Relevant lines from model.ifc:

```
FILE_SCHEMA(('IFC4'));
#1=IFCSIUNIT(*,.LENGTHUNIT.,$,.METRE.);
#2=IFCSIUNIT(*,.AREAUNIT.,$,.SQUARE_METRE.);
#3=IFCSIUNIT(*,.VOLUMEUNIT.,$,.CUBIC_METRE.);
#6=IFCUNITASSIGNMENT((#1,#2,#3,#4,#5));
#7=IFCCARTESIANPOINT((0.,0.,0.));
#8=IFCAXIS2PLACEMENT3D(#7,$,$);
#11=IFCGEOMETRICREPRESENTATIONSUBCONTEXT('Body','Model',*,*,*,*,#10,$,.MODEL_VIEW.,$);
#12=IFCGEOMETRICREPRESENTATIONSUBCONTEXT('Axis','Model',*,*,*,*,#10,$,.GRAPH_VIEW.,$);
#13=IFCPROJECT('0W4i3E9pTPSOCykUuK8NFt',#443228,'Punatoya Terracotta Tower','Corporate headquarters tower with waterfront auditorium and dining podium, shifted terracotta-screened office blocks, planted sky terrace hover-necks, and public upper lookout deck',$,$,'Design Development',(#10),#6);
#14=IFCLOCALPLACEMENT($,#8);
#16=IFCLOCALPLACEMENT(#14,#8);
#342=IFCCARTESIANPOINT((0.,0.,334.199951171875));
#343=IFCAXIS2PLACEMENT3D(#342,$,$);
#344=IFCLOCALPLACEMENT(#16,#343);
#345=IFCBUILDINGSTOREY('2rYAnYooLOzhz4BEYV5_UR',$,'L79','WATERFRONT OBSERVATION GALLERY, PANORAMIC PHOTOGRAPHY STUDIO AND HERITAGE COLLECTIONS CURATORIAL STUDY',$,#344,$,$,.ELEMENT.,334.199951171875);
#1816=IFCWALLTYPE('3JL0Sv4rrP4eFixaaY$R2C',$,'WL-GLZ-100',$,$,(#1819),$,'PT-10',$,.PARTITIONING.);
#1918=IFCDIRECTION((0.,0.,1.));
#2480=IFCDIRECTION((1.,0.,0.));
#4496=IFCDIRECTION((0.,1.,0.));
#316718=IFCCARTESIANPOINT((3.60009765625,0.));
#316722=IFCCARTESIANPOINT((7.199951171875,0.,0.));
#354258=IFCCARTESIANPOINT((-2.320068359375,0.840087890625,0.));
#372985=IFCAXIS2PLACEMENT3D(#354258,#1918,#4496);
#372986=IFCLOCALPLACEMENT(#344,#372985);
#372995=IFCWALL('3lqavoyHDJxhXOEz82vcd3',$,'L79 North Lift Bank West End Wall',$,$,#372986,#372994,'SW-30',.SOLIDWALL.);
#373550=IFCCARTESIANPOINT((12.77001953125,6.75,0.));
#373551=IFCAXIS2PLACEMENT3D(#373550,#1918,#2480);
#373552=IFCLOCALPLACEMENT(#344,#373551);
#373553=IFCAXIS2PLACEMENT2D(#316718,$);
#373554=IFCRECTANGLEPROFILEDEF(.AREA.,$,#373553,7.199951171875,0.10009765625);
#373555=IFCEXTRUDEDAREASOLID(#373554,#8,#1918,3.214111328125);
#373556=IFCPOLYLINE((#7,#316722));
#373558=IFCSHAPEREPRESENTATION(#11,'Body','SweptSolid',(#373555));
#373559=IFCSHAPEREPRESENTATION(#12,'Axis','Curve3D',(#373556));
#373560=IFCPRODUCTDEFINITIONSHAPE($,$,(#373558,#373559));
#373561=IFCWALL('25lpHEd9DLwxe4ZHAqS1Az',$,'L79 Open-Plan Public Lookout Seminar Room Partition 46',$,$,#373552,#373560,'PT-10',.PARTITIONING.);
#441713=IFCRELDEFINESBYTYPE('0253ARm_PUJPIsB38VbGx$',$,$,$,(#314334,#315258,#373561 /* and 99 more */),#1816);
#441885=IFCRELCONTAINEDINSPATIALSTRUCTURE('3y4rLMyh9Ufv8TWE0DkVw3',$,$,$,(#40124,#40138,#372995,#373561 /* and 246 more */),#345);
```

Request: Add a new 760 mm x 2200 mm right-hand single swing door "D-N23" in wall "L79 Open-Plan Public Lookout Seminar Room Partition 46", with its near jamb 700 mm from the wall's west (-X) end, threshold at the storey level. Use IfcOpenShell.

```python
import numpy as np
import ifcopenshell
import ifcopenshell.api.feature
import ifcopenshell.api.geometry
import ifcopenshell.api.root
import ifcopenshell.api.spatial
import ifcopenshell.geom
import ifcopenshell.util.element
import ifcopenshell.util.placement
import ifcopenshell.util.representation
import ifcopenshell.util.shape
import ifcopenshell.util.unit

model = ifcopenshell.open("model.ifc")
unit_scale = ifcopenshell.util.unit.calculate_unit_scale(model)
settings = ifcopenshell.geom.settings()


def volume(element):
    """Net volume in cubic metres, openings subtracted."""
    shape = ifcopenshell.geom.create_shape(settings, element)
    return ifcopenshell.util.shape.get_volume(shape.geometry)


wall = model.by_guid("25lpHEd9DLwxe4ZHAqS1Az")
storey = ifcopenshell.util.element.get_container(wall, ifc_class="IfcBuildingStorey")
context = ifcopenshell.util.representation.get_context(model, "Model", "Body", "MODEL_VIEW")
before = volume(wall)

width, height, from_end, sill = 0.76, 2.2, 0.7, 0.0  # metres

# The wall runs along its own X axis, and the end named is its -X end.
wall_shape = ifcopenshell.geom.create_shape(settings, wall)
x, y, z = ifcopenshell.util.shape.get_vertices(wall_shape.geometry).T
start = x.min() + from_end
face, thickness = float(y.min()), float(y.max() - y.min())
wall_matrix = ifcopenshell.util.placement.get_local_placement(wall.ObjectPlacement)
level = ifcopenshell.util.placement.get_local_placement(storey.ObjectPlacement)[2, 3]


def in_wall(x, y):
    """Placement at x, y metres in the wall's axes, at sill height."""
    matrix = wall_matrix.copy()
    matrix[:, 3] = wall_matrix @ np.array([x / unit_scale, y / unit_scale, 0.0, 1.0])
    matrix[2, 3] = level + sill / unit_scale
    return matrix


# Opening: a box that overshoots both wall faces by 50 mm.
opening = ifcopenshell.api.root.create_entity(model, ifc_class="IfcOpeningElement", predefined_type="OPENING")
box = ifcopenshell.api.geometry.add_wall_representation(
    model, context=context, length=width, height=height, thickness=thickness + 0.1
)
ifcopenshell.api.geometry.assign_representation(model, product=opening, representation=box)
ifcopenshell.api.geometry.edit_object_placement(model, product=opening, matrix=in_wall(start, face - 0.05), is_si=False)
ifcopenshell.api.feature.add_feature(model, feature=opening, element=wall)

door = ifcopenshell.api.root.create_entity(model, ifc_class="IfcDoor", name="D-N23", predefined_type="DOOR")
door.OverallWidth, door.OverallHeight = width / unit_scale, height / unit_scale
door.OperationType = "SINGLE_SWING_RIGHT"
body = ifcopenshell.api.geometry.add_door_representation(
    model,
    context=context,
    overall_width=door.OverallWidth,
    overall_height=door.OverallHeight,
    operation_type="SINGLE_SWING_RIGHT",
    lining_properties={"LiningDepth": thickness / unit_scale, "ThresholdDepth": thickness / unit_scale},
)
ifcopenshell.api.geometry.assign_representation(model, product=door, representation=body)
ifcopenshell.api.spatial.assign_container(model, products=[door], relating_structure=storey)
ifcopenshell.api.feature.add_filling(model, opening=opening, element=door)

# The lining spans the wall, so the door starts at the wall face.
ifcopenshell.api.geometry.edit_object_placement(model, product=door, matrix=in_wall(start, face), is_si=False)

after = volume(wall)

print(f"wall volume {before:.3f} -> {after:.3f} m3")

model.write("model-out.ifc")
```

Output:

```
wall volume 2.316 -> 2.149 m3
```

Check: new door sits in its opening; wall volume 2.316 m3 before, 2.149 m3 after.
